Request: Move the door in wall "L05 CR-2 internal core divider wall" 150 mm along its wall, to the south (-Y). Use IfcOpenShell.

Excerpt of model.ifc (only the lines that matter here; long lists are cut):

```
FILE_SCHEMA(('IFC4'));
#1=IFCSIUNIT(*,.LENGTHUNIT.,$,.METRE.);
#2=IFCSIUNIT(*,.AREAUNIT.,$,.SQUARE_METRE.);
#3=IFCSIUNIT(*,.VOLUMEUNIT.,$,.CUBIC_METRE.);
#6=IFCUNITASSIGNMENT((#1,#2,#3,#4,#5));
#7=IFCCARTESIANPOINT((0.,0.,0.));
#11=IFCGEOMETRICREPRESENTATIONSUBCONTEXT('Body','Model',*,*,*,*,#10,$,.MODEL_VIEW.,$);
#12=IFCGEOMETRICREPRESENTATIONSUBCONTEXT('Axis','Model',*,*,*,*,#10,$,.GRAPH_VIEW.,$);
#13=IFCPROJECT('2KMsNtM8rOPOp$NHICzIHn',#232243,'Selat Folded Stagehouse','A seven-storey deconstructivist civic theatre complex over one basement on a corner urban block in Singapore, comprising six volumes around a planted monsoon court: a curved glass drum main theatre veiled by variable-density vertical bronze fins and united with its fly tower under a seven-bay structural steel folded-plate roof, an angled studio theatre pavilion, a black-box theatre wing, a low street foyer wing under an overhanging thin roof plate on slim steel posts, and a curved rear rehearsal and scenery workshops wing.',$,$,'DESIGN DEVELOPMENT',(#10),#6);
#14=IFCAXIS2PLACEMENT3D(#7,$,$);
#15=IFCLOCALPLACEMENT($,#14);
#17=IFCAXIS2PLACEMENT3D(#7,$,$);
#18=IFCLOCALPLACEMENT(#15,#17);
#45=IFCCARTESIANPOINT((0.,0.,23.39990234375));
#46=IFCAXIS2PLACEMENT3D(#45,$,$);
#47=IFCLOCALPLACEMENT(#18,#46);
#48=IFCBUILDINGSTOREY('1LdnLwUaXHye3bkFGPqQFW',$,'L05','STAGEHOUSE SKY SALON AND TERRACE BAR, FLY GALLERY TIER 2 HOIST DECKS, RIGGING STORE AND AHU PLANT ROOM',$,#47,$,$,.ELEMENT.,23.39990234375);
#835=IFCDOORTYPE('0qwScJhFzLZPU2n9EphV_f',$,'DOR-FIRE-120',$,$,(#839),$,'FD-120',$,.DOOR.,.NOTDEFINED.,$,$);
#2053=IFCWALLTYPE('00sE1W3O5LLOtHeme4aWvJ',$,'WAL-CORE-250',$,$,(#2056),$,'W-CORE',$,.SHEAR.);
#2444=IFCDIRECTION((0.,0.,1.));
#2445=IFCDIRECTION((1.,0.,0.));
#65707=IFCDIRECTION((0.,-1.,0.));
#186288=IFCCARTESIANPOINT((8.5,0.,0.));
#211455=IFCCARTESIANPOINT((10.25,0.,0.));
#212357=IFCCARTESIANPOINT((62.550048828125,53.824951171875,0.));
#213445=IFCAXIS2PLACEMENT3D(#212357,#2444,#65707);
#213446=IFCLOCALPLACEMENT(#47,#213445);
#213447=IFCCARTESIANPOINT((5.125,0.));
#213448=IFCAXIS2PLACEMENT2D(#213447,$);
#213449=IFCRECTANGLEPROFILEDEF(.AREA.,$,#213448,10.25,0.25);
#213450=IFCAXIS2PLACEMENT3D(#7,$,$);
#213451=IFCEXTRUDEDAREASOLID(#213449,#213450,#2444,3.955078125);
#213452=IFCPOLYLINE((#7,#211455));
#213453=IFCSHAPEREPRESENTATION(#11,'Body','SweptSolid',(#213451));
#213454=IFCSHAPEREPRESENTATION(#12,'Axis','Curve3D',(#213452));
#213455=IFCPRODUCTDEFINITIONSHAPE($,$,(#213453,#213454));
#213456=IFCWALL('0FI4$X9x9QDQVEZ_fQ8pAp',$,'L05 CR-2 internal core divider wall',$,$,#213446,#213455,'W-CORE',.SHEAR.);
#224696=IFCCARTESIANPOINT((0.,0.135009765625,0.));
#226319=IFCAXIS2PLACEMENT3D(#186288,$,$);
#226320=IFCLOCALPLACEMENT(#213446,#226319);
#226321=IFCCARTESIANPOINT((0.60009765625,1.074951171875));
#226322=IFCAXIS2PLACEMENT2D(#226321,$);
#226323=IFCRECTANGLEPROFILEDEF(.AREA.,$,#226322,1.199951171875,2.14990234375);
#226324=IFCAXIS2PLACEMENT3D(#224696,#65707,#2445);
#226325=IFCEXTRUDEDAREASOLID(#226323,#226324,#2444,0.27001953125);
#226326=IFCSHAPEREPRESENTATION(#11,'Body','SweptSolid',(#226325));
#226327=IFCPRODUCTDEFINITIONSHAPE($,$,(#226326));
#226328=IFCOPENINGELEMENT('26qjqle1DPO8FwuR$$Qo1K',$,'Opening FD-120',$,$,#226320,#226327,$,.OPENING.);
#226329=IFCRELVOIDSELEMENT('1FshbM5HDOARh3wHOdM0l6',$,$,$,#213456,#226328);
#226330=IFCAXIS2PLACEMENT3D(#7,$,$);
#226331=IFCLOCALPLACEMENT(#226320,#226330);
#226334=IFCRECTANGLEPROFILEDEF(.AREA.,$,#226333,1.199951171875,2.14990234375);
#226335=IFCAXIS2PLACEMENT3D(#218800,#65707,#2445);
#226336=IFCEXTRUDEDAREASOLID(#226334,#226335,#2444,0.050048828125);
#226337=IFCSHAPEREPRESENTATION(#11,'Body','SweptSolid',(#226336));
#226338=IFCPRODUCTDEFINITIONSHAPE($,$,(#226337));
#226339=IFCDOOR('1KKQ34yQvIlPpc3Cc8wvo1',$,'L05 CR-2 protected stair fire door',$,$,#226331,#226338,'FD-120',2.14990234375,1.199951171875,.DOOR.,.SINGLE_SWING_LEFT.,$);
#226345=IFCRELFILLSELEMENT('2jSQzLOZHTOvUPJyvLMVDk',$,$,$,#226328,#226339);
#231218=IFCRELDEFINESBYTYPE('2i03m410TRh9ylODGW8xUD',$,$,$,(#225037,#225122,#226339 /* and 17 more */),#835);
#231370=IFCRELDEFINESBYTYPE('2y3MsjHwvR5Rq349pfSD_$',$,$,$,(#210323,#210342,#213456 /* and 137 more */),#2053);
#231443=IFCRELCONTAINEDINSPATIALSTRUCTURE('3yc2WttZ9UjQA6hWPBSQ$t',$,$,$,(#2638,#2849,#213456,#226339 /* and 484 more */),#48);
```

```python
import ifcopenshell
import ifcopenshell.api.geometry
import ifcopenshell.util.placement
import ifcopenshell.util.unit

model = ifcopenshell.open("model.ifc")
unit_scale = ifcopenshell.util.unit.calculate_unit_scale(model)

door = model.by_guid("1KKQ34yQvIlPpc3Cc8wvo1")
opening = door.FillsVoids[0].RelatingOpeningElement
wall = opening.VoidsElements[0].RelatingBuildingElement

wall_matrix = ifcopenshell.util.placement.get_local_placement(wall.ObjectPlacement)
shift = wall_matrix[:3, 0] * 0.15 / unit_scale
before = ifcopenshell.util.placement.get_local_placement(door.ObjectPlacement)[:3, 3].copy()

# The door is placed relative to its opening, so it follows when the opening moves.
matrix = ifcopenshell.util.placement.get_local_placement(opening.ObjectPlacement)
matrix[:3, 3] += shift
ifcopenshell.api.geometry.edit_object_placement(
    model, product=opening, matrix=matrix, is_si=False, should_transform_children=True
)

after = ifcopenshell.util.placement.get_local_placement(door.ObjectPlacement)[:3, 3]
print("door moved by", (after - before).round(3) + 0.0)

model.write("model_edited.ifc")
```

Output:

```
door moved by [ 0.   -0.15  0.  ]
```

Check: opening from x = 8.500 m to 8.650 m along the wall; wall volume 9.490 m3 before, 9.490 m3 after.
